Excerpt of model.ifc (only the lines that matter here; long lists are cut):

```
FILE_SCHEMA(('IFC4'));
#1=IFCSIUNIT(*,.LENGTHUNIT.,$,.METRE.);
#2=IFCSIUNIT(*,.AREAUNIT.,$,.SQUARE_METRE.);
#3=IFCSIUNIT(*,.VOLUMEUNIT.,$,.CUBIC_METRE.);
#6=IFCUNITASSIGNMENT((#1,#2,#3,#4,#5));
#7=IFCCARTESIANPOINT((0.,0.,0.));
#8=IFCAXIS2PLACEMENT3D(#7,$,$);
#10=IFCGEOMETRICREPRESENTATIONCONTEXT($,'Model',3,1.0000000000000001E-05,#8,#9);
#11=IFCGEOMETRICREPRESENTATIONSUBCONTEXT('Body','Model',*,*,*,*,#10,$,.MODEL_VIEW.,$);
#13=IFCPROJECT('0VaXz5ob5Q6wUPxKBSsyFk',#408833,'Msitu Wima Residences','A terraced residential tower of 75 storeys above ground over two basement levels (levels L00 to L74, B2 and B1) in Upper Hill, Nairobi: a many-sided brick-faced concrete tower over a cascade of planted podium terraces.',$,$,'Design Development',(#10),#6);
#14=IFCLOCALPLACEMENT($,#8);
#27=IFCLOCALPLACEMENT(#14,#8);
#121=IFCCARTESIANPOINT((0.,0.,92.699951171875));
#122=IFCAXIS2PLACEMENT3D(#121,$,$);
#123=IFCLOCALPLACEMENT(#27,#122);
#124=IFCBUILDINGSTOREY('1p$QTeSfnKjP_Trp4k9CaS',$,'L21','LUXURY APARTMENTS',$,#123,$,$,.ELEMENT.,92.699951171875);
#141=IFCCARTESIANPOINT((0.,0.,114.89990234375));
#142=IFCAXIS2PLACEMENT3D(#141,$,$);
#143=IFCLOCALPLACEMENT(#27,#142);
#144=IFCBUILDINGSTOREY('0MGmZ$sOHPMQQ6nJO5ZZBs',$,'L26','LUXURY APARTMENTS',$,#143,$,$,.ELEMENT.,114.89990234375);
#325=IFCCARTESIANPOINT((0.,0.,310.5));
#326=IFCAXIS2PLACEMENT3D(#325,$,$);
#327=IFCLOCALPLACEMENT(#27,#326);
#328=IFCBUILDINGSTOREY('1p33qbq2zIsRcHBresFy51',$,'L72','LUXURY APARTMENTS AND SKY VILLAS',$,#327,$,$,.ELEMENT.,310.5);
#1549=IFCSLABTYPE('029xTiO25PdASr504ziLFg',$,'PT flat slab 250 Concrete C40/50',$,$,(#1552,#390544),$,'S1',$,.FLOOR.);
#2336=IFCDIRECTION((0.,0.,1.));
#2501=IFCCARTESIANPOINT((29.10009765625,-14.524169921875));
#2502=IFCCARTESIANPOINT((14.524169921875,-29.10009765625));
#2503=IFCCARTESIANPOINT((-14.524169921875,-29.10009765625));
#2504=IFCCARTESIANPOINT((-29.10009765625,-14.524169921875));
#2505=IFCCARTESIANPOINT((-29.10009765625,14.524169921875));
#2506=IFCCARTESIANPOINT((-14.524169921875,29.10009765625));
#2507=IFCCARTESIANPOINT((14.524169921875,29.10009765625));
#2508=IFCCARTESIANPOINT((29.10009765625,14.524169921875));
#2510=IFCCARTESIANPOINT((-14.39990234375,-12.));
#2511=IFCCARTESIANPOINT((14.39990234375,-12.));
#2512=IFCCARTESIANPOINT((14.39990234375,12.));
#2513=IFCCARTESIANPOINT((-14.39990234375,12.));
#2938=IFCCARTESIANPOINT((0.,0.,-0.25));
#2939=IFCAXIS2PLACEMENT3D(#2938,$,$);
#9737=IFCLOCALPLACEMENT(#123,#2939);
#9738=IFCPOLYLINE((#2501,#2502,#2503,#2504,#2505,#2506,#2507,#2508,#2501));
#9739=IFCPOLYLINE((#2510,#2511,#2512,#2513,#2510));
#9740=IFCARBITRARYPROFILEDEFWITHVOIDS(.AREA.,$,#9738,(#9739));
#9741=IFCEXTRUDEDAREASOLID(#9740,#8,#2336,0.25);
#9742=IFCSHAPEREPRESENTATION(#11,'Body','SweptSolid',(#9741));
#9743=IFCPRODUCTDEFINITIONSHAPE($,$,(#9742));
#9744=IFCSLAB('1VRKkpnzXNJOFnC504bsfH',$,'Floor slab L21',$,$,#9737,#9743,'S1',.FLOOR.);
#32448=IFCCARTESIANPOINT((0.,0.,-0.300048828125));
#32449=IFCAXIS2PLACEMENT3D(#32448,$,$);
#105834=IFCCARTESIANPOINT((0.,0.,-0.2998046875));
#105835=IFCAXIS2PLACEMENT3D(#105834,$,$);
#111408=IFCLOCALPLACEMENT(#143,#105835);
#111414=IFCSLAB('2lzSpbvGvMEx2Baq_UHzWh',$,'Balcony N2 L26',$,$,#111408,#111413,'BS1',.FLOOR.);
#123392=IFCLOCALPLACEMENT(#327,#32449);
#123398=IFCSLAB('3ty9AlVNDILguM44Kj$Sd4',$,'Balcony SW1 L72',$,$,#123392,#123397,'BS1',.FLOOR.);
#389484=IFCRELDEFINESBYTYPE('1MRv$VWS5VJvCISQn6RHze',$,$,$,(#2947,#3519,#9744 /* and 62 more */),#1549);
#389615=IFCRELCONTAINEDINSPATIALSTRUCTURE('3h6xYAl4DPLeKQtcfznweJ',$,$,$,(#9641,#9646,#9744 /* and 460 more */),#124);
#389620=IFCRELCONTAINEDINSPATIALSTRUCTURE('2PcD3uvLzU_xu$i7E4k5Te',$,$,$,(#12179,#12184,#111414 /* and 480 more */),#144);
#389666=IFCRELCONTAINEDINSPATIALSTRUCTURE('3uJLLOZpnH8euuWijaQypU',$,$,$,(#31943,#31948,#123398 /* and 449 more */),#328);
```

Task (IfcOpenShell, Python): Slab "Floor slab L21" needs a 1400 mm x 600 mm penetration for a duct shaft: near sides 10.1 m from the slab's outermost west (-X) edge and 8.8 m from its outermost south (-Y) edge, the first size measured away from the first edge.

```python
import numpy as np
import ifcopenshell
import ifcopenshell.api.feature
import ifcopenshell.api.geometry
import ifcopenshell.api.root
import ifcopenshell.geom
import ifcopenshell.util.placement
import ifcopenshell.util.representation
import ifcopenshell.util.shape
import ifcopenshell.util.unit

model = ifcopenshell.open("model.ifc")
unit_scale = ifcopenshell.util.unit.calculate_unit_scale(model)
settings = ifcopenshell.geom.settings()


def volume(element):
    """Net volume in cubic metres, openings subtracted."""
    shape = ifcopenshell.geom.create_shape(settings, element)
    return ifcopenshell.util.shape.get_volume(shape.geometry)


slab = model.by_id(9744)
before = volume(slab)

# Extent in the slab's own axes, in metres. The edges named are its -X and -Y sides.
slab_shape = ifcopenshell.geom.create_shape(settings, slab)
vertices = ifcopenshell.util.shape.get_vertices(slab_shape.geometry)
x_min, y_min, bottom = vertices.min(axis=0)
top = vertices[:, 2].max()

opening = ifcopenshell.api.root.create_entity(model, ifc_class="IfcOpeningElement", name="Duct shaft opening", predefined_type="OPENING")
context = ifcopenshell.util.representation.get_context(model, "Model", "Body", "MODEL_VIEW")
width, depth = 1.4, 0.6
outline = [(0.0, 0.0), (width, 0.0), (width, depth), (0.0, depth), (0.0, 0.0)]
# Overshoot both faces by 50 mm so the cut is clean.
shape = ifcopenshell.api.geometry.add_slab_representation(
    model, context=context, depth=top - bottom + 0.1, polyline=outline
)
ifcopenshell.api.geometry.assign_representation(model, product=opening, representation=shape)

matrix = ifcopenshell.util.placement.get_local_placement(slab.ObjectPlacement)
matrix[:, 3] = matrix @ np.append(np.array([x_min + 10.1, y_min + 8.8, bottom - 0.05]) / unit_scale, 1.0)
ifcopenshell.api.geometry.edit_object_placement(model, product=opening, matrix=matrix, is_si=False)
ifcopenshell.api.feature.add_feature(model, feature=opening, element=slab)

after = volume(slab)

print(f"slab volume {before:.3f} -> {after:.3f} m3")

model.write("model-out.ifc")
```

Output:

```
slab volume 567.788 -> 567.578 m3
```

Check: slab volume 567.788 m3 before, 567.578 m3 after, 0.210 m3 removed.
